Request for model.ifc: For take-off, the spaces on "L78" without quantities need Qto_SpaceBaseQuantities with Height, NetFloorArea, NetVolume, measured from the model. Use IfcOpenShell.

First a look at what the model holds.

```python
import ifcopenshell
import ifcopenshell.util.element
import ifcopenshell.util.unit

model = ifcopenshell.open("model.ifc")
print(model.schema)
for unit_type in ("LENGTHUNIT", "AREAUNIT", "VOLUMEUNIT"):
    print(unit_type, ifcopenshell.util.unit.calculate_unit_scale(model, unit_type))
storey = next(s for s in model.by_type("IfcBuildingStorey") if s.Name == "L78")
spaces = [e for e in ifcopenshell.util.element.get_decomposition(storey) if e.is_a("IfcSpace")]
for e in sorted(spaces, key=lambda e: e.id()):
    print(e.id(), e.is_a(), e.Name, list(ifcopenshell.util.element.get_psets(e, qtos_only=True)), sep=" | ")
```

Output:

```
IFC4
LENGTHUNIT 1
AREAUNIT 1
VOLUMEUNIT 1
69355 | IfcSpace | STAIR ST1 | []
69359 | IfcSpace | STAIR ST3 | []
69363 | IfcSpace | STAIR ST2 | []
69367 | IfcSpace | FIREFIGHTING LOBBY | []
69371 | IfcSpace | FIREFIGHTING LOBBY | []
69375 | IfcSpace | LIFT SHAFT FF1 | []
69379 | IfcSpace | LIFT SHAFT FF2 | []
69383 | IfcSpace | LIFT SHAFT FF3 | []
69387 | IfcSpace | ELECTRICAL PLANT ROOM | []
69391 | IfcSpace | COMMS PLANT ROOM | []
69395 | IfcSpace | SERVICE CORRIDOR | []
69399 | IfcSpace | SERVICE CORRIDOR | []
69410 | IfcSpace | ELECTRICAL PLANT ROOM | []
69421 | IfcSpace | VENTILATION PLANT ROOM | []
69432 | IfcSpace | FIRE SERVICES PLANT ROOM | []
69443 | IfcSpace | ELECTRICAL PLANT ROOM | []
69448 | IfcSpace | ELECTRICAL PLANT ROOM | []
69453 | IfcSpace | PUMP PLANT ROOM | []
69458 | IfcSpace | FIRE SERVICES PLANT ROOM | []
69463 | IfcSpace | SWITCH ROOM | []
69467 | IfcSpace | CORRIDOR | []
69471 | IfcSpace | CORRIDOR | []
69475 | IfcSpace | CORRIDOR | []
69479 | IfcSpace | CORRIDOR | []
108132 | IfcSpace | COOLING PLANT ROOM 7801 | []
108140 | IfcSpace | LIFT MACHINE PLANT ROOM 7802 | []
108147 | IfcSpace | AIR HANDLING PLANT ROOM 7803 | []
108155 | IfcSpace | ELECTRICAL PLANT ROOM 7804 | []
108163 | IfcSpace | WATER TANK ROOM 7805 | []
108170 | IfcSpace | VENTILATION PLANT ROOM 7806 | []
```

```python
import ifcopenshell
import ifcopenshell.api.pset
import ifcopenshell.geom
import ifcopenshell.util.element
import ifcopenshell.util.shape
import ifcopenshell.util.unit

model = ifcopenshell.open("model.ifc")
unit_scale = ifcopenshell.util.unit.calculate_unit_scale(model)
area_scale = ifcopenshell.util.unit.calculate_unit_scale(model, "AREAUNIT")
volume_scale = ifcopenshell.util.unit.calculate_unit_scale(model, "VOLUMEUNIT")
settings = ifcopenshell.geom.settings()

storey = next(s for s in model.by_type("IfcBuildingStorey") if s.Name == "L78")
spaces = [e for e in ifcopenshell.util.element.get_decomposition(storey) if e.is_a("IfcSpace")]

for e in sorted(spaces, key=lambda e: e.id()):
    if ifcopenshell.util.element.get_psets(e, qtos_only=True, should_inherit=False):
        continue
    # Geometry comes back in metres, in the element's own axes.
    shape = ifcopenshell.geom.create_shape(settings, e)
    values = {
        "Height": ifcopenshell.util.shape.get_z(shape.geometry) / unit_scale,
        "NetFloorArea": ifcopenshell.util.shape.get_footprint_area(shape.geometry) / area_scale,
        "NetVolume": ifcopenshell.util.shape.get_volume(shape.geometry) / volume_scale,
    }
    qto = ifcopenshell.api.pset.add_qto(model, product=e, name="Qto_SpaceBaseQuantities")
    ifcopenshell.api.pset.edit_qto(model, qto=qto, properties=values)
    print(e.id(), {k: round(v, 3) for k, v in values.items()})

model.write("model_edited.ifc")
```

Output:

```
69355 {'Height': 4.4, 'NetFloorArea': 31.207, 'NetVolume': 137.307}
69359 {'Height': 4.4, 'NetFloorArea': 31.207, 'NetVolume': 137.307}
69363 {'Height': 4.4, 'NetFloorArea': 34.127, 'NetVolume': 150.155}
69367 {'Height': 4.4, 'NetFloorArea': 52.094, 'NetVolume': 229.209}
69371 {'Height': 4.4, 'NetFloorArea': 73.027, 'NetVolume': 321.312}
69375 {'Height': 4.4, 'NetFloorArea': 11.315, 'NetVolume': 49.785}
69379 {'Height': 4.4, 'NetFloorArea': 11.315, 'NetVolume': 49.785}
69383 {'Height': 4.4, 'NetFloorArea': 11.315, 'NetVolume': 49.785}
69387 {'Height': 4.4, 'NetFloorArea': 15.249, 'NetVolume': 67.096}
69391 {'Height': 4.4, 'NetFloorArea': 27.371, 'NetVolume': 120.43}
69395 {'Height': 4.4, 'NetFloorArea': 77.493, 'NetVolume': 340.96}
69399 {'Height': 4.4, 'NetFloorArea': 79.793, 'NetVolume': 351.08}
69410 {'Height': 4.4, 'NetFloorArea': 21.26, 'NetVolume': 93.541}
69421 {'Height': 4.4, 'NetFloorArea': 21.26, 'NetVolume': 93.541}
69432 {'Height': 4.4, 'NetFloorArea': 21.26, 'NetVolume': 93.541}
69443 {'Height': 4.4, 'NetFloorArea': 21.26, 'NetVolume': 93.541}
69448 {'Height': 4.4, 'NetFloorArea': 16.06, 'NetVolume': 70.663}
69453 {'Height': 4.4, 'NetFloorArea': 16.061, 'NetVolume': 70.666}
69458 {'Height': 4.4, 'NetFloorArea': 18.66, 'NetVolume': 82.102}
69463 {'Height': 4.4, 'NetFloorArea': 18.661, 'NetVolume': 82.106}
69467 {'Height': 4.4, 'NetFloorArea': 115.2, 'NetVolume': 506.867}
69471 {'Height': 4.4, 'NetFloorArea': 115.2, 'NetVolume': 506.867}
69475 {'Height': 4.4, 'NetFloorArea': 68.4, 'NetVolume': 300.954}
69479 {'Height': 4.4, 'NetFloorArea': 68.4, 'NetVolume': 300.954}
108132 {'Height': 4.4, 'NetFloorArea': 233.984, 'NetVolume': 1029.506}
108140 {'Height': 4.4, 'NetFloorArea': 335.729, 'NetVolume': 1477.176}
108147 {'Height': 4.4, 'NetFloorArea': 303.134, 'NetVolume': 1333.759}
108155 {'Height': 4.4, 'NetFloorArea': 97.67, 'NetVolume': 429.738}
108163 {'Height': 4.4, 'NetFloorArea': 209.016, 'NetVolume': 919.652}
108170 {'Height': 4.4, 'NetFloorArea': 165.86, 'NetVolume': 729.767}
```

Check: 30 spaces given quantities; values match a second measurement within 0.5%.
